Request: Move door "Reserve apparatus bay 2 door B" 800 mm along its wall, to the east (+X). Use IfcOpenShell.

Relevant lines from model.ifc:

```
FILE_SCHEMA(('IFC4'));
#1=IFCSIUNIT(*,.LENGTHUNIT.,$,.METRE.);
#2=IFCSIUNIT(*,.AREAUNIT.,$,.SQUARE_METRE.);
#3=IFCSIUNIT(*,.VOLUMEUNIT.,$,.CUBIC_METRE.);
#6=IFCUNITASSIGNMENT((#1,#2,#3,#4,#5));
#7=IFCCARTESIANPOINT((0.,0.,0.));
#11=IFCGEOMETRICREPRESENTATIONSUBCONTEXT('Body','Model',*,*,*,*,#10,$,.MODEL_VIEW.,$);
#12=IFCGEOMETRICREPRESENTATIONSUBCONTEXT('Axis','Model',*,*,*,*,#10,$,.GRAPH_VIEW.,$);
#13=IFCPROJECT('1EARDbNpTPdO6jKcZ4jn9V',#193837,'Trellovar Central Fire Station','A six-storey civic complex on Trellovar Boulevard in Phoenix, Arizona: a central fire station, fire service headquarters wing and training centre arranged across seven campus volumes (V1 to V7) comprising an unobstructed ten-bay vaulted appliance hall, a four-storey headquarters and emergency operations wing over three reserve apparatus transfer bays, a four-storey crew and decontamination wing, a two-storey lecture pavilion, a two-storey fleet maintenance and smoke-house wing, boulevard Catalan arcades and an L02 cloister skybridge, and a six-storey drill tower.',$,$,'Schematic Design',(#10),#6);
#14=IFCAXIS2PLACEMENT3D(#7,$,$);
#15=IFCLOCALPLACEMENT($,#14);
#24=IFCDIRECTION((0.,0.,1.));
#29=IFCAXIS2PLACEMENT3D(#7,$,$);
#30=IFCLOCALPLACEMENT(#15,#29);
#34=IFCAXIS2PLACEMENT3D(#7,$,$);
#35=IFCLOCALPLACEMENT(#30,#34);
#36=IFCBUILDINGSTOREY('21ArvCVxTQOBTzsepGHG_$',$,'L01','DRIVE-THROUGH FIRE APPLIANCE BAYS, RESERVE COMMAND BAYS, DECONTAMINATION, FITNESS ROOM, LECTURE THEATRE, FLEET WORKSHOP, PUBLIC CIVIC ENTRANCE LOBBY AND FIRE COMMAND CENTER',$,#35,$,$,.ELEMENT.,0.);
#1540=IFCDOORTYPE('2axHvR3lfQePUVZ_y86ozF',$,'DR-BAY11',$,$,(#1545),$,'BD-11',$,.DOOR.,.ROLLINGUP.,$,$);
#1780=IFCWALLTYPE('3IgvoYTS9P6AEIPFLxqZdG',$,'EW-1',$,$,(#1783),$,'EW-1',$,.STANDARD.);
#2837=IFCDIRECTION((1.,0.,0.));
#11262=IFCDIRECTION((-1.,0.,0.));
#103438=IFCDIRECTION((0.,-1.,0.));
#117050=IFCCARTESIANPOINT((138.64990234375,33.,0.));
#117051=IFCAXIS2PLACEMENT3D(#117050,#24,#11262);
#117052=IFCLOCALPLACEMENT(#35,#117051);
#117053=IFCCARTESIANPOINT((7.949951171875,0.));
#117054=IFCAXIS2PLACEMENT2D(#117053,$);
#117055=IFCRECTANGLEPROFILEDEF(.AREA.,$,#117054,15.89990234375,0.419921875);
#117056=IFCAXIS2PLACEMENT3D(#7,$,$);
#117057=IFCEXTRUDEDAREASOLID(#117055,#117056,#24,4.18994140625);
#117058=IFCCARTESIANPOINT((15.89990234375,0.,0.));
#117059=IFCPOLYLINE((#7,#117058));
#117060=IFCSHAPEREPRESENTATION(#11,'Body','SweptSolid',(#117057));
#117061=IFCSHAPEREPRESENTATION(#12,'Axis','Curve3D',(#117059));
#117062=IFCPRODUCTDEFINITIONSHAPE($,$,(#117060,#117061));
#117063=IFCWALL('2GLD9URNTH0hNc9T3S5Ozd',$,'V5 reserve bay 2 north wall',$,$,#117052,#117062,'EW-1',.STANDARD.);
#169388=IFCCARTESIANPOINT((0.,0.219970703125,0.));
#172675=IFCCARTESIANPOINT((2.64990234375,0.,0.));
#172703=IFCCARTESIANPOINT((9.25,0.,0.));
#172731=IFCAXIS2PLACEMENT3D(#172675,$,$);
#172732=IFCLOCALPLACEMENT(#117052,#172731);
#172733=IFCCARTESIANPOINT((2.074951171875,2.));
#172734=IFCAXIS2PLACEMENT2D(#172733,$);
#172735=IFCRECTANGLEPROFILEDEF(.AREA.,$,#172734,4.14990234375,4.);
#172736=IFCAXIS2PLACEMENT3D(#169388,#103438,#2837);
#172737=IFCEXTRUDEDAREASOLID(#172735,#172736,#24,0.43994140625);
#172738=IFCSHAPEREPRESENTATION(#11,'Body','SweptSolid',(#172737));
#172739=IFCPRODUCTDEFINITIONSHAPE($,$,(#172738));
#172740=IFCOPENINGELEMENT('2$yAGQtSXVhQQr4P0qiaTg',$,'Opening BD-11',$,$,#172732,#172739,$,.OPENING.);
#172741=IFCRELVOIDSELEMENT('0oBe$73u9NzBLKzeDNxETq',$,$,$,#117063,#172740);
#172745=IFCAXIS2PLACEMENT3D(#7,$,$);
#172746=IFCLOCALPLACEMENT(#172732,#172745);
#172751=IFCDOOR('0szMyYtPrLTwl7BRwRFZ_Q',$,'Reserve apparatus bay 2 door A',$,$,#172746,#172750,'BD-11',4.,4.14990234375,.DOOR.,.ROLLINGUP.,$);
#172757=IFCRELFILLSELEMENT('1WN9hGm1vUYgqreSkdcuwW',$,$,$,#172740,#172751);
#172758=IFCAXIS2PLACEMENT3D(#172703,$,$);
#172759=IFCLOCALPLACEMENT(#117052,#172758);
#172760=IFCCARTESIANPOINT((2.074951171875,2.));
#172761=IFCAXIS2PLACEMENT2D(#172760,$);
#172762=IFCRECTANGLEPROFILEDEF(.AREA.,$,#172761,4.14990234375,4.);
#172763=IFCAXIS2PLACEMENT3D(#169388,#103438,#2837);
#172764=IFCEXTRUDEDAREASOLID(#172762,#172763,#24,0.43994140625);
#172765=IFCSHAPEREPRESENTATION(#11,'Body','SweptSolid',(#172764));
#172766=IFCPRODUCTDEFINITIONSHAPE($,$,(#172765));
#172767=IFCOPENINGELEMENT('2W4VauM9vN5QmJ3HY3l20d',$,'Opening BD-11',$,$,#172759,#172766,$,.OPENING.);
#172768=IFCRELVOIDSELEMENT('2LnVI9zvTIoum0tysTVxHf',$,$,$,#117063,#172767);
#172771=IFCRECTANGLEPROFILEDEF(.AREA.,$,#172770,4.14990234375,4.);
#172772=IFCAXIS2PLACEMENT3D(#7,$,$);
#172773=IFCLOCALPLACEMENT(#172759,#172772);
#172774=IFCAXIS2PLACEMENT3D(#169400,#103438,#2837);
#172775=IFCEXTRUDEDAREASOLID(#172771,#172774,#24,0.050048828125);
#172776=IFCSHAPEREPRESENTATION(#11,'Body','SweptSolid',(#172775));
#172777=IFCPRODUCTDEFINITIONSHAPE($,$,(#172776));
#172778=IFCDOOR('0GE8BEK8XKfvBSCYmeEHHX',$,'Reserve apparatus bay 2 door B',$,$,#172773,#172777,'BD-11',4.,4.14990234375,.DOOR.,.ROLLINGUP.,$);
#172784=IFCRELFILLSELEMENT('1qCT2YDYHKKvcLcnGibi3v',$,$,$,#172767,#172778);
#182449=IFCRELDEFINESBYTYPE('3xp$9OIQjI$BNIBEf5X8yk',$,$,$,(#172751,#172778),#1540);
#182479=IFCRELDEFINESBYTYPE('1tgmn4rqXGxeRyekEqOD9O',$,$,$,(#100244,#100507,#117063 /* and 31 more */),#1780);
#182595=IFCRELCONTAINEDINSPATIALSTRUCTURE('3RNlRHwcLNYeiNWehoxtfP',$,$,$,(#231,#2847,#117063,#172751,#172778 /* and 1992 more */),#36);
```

```python
import ifcopenshell
import ifcopenshell.api.geometry
import ifcopenshell.util.placement

model = ifcopenshell.open("model.ifc")

door = model.by_guid("0GE8BEK8XKfvBSCYmeEHHX")
opening = door.FillsVoids[0].RelatingOpeningElement
wall = opening.VoidsElements[0].RelatingBuildingElement

wall_matrix = ifcopenshell.util.placement.get_local_placement(wall.ObjectPlacement)
shift = wall_matrix[:3, 0] * -0.8
before = ifcopenshell.util.placement.get_local_placement(door.ObjectPlacement)[:3, 3].copy()

# The door is placed relative to its opening, so it follows when the opening moves.
matrix = ifcopenshell.util.placement.get_local_placement(opening.ObjectPlacement)
matrix[:3, 3] += shift
ifcopenshell.api.geometry.edit_object_placement(
    model, product=opening, matrix=matrix, is_si=False, should_transform_children=True
)

after = ifcopenshell.util.placement.get_local_placement(door.ObjectPlacement)[:3, 3]
print("door moved by", (after - before).round(3) + 0.0)

model.write("model_rev.ifc")
```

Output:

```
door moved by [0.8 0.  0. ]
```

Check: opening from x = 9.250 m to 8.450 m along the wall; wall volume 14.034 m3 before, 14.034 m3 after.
